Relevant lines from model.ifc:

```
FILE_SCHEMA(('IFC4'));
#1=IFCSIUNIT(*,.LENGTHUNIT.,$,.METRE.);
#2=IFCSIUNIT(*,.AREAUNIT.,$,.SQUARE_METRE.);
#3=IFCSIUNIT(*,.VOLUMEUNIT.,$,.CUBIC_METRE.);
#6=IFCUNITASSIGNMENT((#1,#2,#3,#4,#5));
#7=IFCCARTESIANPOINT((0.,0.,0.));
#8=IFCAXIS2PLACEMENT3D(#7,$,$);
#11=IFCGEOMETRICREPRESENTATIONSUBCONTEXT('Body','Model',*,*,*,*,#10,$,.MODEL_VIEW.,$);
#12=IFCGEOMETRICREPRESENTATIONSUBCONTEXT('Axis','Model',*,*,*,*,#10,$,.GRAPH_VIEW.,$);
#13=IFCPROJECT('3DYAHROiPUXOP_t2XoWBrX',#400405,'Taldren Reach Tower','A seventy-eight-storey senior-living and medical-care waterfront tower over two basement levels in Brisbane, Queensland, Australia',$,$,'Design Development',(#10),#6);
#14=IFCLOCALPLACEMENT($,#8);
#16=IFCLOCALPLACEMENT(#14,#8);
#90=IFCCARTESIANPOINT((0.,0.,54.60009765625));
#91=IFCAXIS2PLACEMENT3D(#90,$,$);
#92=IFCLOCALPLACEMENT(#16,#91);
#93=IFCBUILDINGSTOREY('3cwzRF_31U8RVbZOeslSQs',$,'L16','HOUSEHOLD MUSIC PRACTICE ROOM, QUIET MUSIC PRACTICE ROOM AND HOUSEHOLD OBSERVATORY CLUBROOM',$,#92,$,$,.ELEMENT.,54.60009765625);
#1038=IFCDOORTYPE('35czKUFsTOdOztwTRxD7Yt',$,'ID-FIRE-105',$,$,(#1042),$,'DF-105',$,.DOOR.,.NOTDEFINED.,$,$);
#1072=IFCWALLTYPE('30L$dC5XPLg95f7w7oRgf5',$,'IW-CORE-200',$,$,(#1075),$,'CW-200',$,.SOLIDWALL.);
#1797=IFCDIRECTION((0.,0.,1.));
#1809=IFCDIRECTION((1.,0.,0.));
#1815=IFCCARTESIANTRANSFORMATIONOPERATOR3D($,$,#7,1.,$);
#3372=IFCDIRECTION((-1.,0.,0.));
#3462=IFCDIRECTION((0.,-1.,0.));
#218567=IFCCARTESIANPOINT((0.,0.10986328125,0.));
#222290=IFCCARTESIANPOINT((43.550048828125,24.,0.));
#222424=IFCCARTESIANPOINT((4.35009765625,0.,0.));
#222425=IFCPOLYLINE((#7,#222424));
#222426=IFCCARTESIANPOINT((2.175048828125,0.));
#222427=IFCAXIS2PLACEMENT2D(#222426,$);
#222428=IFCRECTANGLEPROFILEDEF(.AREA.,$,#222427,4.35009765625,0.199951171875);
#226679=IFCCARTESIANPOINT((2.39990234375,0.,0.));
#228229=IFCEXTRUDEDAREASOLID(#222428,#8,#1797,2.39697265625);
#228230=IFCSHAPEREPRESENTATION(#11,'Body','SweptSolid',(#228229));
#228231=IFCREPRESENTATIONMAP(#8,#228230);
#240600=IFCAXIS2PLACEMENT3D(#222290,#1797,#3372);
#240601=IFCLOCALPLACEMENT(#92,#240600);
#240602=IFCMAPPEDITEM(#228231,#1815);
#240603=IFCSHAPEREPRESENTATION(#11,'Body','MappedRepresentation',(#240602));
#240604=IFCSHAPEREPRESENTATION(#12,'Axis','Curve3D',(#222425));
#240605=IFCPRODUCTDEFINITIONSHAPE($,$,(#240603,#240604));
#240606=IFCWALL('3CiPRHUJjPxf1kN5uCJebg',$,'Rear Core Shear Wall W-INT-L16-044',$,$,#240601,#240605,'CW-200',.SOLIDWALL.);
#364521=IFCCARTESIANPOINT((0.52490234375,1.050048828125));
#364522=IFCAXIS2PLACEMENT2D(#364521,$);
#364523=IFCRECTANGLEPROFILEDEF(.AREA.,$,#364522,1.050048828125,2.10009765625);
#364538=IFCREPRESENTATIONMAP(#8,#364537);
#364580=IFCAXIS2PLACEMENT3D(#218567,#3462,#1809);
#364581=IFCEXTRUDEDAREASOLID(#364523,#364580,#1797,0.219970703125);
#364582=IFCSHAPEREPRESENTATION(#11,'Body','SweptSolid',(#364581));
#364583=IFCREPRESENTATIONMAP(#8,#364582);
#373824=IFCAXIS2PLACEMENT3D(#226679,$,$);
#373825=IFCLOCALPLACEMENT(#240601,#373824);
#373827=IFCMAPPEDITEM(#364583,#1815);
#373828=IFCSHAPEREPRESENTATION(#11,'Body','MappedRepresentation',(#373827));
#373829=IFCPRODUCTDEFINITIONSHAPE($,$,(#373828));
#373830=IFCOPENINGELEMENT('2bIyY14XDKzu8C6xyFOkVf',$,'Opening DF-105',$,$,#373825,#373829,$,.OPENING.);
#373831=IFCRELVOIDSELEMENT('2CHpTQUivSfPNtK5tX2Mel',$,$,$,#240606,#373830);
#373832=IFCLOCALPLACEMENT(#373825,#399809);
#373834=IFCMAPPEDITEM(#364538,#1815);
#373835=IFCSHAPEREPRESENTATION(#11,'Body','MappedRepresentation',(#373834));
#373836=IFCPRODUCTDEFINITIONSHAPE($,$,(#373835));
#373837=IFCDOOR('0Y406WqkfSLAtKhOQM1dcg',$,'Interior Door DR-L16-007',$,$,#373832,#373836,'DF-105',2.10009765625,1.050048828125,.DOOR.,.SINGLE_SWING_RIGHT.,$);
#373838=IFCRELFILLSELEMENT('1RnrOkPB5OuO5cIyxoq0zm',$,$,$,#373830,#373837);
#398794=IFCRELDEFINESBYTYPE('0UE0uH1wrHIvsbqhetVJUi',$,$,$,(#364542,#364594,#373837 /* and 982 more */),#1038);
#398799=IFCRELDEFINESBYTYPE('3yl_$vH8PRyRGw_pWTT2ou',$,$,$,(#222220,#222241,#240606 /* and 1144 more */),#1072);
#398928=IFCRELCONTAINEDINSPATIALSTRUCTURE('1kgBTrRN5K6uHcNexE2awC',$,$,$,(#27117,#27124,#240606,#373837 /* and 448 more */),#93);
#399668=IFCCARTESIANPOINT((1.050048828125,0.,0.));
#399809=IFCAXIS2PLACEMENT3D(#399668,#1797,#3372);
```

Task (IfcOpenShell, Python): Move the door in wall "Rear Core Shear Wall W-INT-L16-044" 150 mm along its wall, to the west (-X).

```python
import ifcopenshell
import ifcopenshell.api.geometry
import ifcopenshell.util.placement

model = ifcopenshell.open("model.ifc")

door = model.by_id(373837)
opening = door.FillsVoids[0].RelatingOpeningElement
wall = opening.VoidsElements[0].RelatingBuildingElement

wall_matrix = ifcopenshell.util.placement.get_local_placement(wall.ObjectPlacement)
shift = wall_matrix[:3, 0] * 0.15
before = ifcopenshell.util.placement.get_local_placement(door.ObjectPlacement)[:3, 3].copy()

# The door is placed relative to its opening, so it follows when the opening moves.
matrix = ifcopenshell.util.placement.get_local_placement(opening.ObjectPlacement)
matrix[:3, 3] += shift
ifcopenshell.api.geometry.edit_object_placement(
    model, product=opening, matrix=matrix, is_si=False, should_transform_children=True
)

after = ifcopenshell.util.placement.get_local_placement(door.ObjectPlacement)[:3, 3]
print("door moved by", (after - before).round(3) + 0.0)

model.write("model_rev.ifc")
```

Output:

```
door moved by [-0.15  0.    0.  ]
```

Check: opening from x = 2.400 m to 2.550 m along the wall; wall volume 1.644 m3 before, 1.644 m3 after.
